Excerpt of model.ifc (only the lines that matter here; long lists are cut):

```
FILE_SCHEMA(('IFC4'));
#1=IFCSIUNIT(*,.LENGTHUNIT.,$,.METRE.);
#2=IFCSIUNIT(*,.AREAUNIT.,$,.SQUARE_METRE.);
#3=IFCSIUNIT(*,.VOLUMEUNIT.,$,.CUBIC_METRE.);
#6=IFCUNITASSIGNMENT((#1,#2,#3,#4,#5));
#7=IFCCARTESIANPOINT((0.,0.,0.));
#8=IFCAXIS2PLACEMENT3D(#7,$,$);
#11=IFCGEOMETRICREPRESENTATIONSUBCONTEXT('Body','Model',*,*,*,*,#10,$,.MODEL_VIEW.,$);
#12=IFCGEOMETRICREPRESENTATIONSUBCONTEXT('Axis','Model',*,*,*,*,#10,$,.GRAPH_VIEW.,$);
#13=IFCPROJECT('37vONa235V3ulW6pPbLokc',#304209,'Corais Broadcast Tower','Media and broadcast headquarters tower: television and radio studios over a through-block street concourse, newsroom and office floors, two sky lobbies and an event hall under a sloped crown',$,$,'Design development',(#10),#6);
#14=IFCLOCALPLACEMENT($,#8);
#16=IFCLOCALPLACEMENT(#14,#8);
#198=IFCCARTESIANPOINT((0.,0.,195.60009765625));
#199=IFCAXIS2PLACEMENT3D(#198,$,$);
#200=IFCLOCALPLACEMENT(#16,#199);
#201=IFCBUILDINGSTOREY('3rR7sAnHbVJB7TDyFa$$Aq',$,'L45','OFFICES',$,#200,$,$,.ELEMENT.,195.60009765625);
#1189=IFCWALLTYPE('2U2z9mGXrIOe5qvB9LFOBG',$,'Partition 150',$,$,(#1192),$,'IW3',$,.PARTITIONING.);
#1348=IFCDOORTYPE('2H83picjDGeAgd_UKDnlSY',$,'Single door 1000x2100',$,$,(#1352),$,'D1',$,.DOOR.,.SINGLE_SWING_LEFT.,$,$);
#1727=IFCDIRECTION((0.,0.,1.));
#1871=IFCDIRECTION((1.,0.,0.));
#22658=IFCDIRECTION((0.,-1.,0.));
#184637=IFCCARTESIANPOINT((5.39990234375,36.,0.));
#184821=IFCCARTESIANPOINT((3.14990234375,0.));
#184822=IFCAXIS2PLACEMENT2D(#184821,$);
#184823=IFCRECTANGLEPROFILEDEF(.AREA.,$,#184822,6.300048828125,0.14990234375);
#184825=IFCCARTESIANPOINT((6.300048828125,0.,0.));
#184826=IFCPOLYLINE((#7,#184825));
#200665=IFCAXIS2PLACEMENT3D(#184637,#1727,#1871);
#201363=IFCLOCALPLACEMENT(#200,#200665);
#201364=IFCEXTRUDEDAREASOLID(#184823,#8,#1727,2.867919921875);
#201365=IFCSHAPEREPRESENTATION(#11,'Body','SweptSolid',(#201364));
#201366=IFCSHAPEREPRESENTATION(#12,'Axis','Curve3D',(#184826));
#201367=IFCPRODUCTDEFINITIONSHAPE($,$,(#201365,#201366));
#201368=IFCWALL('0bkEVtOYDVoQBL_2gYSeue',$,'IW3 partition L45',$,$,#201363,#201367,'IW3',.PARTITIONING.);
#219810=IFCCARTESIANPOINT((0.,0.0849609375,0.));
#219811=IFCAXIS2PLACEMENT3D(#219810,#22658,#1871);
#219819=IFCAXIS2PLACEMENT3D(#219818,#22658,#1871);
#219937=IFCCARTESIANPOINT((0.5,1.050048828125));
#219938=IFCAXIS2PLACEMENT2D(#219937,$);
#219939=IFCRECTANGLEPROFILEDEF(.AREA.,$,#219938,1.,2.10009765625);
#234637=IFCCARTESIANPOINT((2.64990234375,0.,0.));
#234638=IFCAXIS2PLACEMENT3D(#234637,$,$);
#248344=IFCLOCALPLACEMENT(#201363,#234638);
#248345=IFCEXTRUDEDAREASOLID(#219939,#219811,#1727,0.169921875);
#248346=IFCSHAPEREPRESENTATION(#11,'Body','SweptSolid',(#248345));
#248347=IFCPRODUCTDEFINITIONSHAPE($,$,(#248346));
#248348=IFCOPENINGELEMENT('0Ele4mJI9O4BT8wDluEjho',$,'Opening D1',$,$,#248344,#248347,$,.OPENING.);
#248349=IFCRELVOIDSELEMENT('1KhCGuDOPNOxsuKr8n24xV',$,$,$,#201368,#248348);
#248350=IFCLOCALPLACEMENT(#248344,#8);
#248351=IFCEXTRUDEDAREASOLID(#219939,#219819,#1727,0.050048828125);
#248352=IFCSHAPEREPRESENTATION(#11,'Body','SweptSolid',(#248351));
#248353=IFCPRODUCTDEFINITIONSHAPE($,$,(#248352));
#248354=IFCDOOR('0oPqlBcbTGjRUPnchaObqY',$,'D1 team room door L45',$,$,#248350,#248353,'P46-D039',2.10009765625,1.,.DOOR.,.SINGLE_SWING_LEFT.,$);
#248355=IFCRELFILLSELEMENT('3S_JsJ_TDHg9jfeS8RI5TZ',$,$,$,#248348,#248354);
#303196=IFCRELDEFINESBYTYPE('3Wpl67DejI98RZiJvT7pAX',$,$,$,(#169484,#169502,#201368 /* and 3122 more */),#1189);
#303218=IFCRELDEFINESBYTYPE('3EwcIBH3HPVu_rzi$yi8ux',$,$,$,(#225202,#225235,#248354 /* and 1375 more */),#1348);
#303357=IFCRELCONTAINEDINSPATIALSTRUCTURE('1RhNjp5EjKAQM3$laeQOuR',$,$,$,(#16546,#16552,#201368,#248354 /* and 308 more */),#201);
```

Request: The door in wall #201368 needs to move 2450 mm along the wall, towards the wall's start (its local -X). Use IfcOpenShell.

```python
import ifcopenshell
import ifcopenshell.api.geometry
import ifcopenshell.util.placement
import ifcopenshell.util.unit

model = ifcopenshell.open("model.ifc")
unit_scale = ifcopenshell.util.unit.calculate_unit_scale(model)

door = model.by_id(248354)
opening = door.FillsVoids[0].RelatingOpeningElement
wall = opening.VoidsElements[0].RelatingBuildingElement

wall_matrix = ifcopenshell.util.placement.get_local_placement(wall.ObjectPlacement)
shift = wall_matrix[:3, 0] * -2.45 / unit_scale
before = ifcopenshell.util.placement.get_local_placement(door.ObjectPlacement)[:3, 3].copy()

# The door is placed relative to its opening, so it follows when the opening moves.
matrix = ifcopenshell.util.placement.get_local_placement(opening.ObjectPlacement)
matrix[:3, 3] += shift
ifcopenshell.api.geometry.edit_object_placement(
    model, product=opening, matrix=matrix, is_si=False, should_transform_children=True
)

after = ifcopenshell.util.placement.get_local_placement(door.ObjectPlacement)[:3, 3]
print("door moved by", (after - before).round(3) + 0.0)

model.write("model-out.ifc")
```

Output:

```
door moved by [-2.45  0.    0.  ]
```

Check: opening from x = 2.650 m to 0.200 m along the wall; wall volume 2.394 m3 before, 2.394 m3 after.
